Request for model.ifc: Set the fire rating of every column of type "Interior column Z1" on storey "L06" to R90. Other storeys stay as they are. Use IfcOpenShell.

First a look at what the model holds.

```python
import ifcopenshell
import ifcopenshell.util.element

model = ifcopenshell.open("model.ifc")
print(model.schema)
storey = next(s for s in model.by_type("IfcBuildingStorey") if s.Name == "L06")
columns = [e for e in ifcopenshell.util.element.get_decomposition(storey) if e.is_a("IfcColumn")]
seen = {}
for e in columns:
    element_type = ifcopenshell.util.element.get_type(e)
    key = (element_type.Name if element_type != e and element_type else None, ifcopenshell.util.element.get_pset(e, "Pset_ColumnCommon", "FireRating"))
    seen[key] = seen.get(key, 0) + 1
for (name, value), count in sorted(seen.items(), key=str):
    print(count, "x", name, "|", value)
```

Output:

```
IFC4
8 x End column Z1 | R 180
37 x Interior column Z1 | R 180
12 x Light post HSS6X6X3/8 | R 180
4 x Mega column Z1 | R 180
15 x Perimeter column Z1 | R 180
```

```python
import ifcopenshell
import ifcopenshell.api.pset
import ifcopenshell.util.element

model = ifcopenshell.open("model.ifc")

storey = next(s for s in model.by_type("IfcBuildingStorey") if s.Name == "L06")
columns = [e for e in ifcopenshell.util.element.get_decomposition(storey) if e.is_a("IfcColumn")]

count = 0
for e in columns:
    element_type = ifcopenshell.util.element.get_type(e)
    if element_type in (None, e) or element_type.Name != "Interior column Z1":
        continue
    found = ifcopenshell.util.element.get_pset(e, "Pset_ColumnCommon", should_inherit=False)
    if found:
        pset = model.by_id(found["id"])
        if len(ifcopenshell.util.element.get_elements_by_pset(pset)) > 1:
            pset = ifcopenshell.api.pset.unshare_pset(model, products=[e], pset=pset)[0]
    else:
        pset = ifcopenshell.api.pset.add_pset(model, product=e, name="Pset_ColumnCommon")
    ifcopenshell.api.pset.edit_pset(model, pset=pset, properties={"FireRating": "R90"})
    count += 1

print(count, "columns updated")

model.write("model_edited.ifc")
```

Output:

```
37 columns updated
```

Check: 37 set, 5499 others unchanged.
